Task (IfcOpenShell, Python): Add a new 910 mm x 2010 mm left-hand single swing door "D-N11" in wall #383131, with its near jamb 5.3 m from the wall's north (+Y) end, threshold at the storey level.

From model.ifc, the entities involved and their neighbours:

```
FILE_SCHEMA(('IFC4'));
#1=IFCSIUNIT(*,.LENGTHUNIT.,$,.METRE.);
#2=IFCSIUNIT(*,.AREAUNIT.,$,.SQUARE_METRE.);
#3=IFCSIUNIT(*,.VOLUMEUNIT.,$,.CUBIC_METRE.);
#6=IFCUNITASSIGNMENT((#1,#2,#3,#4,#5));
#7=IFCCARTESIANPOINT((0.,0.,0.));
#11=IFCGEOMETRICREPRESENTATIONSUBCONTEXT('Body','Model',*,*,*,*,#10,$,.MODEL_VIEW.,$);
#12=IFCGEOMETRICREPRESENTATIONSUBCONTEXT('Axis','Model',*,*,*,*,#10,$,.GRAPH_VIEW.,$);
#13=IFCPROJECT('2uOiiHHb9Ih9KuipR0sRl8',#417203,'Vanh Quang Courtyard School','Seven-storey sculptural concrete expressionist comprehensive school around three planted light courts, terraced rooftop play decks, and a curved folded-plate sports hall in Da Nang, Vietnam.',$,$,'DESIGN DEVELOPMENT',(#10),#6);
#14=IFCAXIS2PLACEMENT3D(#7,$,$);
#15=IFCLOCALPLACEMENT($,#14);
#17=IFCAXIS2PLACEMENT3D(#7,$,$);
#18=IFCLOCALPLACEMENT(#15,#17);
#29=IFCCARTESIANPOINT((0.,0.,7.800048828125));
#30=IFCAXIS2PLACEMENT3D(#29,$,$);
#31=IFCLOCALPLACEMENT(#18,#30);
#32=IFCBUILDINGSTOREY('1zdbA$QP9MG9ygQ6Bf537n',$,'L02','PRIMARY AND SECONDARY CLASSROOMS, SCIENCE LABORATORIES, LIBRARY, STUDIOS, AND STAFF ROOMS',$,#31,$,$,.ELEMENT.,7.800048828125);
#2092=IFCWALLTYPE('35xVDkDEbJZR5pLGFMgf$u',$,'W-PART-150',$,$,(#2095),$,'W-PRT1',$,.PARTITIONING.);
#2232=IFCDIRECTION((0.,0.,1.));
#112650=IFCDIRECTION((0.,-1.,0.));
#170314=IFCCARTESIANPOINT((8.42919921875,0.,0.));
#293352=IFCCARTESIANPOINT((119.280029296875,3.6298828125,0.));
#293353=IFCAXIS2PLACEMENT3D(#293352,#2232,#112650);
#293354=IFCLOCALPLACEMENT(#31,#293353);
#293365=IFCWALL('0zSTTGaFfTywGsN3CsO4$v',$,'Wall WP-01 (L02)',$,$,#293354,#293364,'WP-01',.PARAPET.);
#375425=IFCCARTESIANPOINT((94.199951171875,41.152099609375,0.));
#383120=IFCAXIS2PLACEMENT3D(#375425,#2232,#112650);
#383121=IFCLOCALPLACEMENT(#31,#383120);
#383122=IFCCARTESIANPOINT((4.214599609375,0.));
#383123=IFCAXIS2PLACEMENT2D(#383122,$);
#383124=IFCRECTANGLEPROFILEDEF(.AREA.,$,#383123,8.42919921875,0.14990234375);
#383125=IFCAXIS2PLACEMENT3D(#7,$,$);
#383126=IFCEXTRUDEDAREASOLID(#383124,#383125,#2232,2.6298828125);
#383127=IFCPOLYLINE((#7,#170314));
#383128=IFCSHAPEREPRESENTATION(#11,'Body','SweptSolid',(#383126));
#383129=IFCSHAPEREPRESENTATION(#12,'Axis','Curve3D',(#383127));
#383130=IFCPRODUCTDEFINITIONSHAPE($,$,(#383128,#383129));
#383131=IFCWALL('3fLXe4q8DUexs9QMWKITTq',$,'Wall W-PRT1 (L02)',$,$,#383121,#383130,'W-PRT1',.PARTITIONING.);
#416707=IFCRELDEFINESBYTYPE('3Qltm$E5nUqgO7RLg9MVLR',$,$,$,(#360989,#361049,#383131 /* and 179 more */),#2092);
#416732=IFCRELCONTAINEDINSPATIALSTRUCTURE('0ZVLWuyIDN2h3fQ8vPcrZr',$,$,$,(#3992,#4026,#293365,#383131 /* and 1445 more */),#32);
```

```python
import numpy as np
import ifcopenshell
import ifcopenshell.api.feature
import ifcopenshell.api.geometry
import ifcopenshell.api.root
import ifcopenshell.api.spatial
import ifcopenshell.geom
import ifcopenshell.util.element
import ifcopenshell.util.placement
import ifcopenshell.util.representation
import ifcopenshell.util.shape
import ifcopenshell.util.unit

model = ifcopenshell.open("model.ifc")
unit_scale = ifcopenshell.util.unit.calculate_unit_scale(model)
settings = ifcopenshell.geom.settings()


def volume(element):
    """Net volume in cubic metres, openings subtracted."""
    shape = ifcopenshell.geom.create_shape(settings, element)
    return ifcopenshell.util.shape.get_volume(shape.geometry)


wall = model.by_guid("3fLXe4q8DUexs9QMWKITTq")
storey = ifcopenshell.util.element.get_container(wall, ifc_class="IfcBuildingStorey")
context = ifcopenshell.util.representation.get_context(model, "Model", "Body", "MODEL_VIEW")
before = volume(wall)

width, height, from_end, sill = 0.91, 2.01, 5.3, 0.0  # metres

# The wall runs along its own X axis, and the end named is its -X end.
wall_shape = ifcopenshell.geom.create_shape(settings, wall)
x, y, z = ifcopenshell.util.shape.get_vertices(wall_shape.geometry).T
start = x.min() + from_end
face, thickness = float(y.min()), float(y.max() - y.min())
wall_matrix = ifcopenshell.util.placement.get_local_placement(wall.ObjectPlacement)
level = ifcopenshell.util.placement.get_local_placement(storey.ObjectPlacement)[2, 3]


def in_wall(x, y):
    """Placement at x, y metres in the wall's axes, at sill height."""
    matrix = wall_matrix.copy()
    matrix[:, 3] = wall_matrix @ np.array([x / unit_scale, y / unit_scale, 0.0, 1.0])
    matrix[2, 3] = level + sill / unit_scale
    return matrix


# Opening: a box that overshoots both wall faces by 50 mm.
opening = ifcopenshell.api.root.create_entity(model, ifc_class="IfcOpeningElement", predefined_type="OPENING")
box = ifcopenshell.api.geometry.add_wall_representation(
    model, context=context, length=width, height=height, thickness=thickness + 0.1
)
ifcopenshell.api.geometry.assign_representation(model, product=opening, representation=box)
ifcopenshell.api.geometry.edit_object_placement(model, product=opening, matrix=in_wall(start, face - 0.05), is_si=False)
ifcopenshell.api.feature.add_feature(model, feature=opening, element=wall)

door = ifcopenshell.api.root.create_entity(model, ifc_class="IfcDoor", name="D-N11", predefined_type="DOOR")
door.OverallWidth, door.OverallHeight = width / unit_scale, height / unit_scale
door.OperationType = "SINGLE_SWING_LEFT"
body = ifcopenshell.api.geometry.add_door_representation(
    model,
    context=context,
    overall_width=door.OverallWidth,
    overall_height=door.OverallHeight,
    operation_type="SINGLE_SWING_LEFT",
    lining_properties={"LiningDepth": thickness / unit_scale, "ThresholdDepth": thickness / unit_scale},
)
ifcopenshell.api.geometry.assign_representation(model, product=door, representation=body)
ifcopenshell.api.spatial.assign_container(model, products=[door], relating_structure=storey)
ifcopenshell.api.feature.add_filling(model, opening=opening, element=door)

# The lining spans the wall, so the door starts at the wall face.
ifcopenshell.api.geometry.edit_object_placement(model, product=door, matrix=in_wall(start, face), is_si=False)

after = volume(wall)

print(f"wall volume {before:.3f} -> {after:.3f} m3")

model.write("model_rev.ifc")
```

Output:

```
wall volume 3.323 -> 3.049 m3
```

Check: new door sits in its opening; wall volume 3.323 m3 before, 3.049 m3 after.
